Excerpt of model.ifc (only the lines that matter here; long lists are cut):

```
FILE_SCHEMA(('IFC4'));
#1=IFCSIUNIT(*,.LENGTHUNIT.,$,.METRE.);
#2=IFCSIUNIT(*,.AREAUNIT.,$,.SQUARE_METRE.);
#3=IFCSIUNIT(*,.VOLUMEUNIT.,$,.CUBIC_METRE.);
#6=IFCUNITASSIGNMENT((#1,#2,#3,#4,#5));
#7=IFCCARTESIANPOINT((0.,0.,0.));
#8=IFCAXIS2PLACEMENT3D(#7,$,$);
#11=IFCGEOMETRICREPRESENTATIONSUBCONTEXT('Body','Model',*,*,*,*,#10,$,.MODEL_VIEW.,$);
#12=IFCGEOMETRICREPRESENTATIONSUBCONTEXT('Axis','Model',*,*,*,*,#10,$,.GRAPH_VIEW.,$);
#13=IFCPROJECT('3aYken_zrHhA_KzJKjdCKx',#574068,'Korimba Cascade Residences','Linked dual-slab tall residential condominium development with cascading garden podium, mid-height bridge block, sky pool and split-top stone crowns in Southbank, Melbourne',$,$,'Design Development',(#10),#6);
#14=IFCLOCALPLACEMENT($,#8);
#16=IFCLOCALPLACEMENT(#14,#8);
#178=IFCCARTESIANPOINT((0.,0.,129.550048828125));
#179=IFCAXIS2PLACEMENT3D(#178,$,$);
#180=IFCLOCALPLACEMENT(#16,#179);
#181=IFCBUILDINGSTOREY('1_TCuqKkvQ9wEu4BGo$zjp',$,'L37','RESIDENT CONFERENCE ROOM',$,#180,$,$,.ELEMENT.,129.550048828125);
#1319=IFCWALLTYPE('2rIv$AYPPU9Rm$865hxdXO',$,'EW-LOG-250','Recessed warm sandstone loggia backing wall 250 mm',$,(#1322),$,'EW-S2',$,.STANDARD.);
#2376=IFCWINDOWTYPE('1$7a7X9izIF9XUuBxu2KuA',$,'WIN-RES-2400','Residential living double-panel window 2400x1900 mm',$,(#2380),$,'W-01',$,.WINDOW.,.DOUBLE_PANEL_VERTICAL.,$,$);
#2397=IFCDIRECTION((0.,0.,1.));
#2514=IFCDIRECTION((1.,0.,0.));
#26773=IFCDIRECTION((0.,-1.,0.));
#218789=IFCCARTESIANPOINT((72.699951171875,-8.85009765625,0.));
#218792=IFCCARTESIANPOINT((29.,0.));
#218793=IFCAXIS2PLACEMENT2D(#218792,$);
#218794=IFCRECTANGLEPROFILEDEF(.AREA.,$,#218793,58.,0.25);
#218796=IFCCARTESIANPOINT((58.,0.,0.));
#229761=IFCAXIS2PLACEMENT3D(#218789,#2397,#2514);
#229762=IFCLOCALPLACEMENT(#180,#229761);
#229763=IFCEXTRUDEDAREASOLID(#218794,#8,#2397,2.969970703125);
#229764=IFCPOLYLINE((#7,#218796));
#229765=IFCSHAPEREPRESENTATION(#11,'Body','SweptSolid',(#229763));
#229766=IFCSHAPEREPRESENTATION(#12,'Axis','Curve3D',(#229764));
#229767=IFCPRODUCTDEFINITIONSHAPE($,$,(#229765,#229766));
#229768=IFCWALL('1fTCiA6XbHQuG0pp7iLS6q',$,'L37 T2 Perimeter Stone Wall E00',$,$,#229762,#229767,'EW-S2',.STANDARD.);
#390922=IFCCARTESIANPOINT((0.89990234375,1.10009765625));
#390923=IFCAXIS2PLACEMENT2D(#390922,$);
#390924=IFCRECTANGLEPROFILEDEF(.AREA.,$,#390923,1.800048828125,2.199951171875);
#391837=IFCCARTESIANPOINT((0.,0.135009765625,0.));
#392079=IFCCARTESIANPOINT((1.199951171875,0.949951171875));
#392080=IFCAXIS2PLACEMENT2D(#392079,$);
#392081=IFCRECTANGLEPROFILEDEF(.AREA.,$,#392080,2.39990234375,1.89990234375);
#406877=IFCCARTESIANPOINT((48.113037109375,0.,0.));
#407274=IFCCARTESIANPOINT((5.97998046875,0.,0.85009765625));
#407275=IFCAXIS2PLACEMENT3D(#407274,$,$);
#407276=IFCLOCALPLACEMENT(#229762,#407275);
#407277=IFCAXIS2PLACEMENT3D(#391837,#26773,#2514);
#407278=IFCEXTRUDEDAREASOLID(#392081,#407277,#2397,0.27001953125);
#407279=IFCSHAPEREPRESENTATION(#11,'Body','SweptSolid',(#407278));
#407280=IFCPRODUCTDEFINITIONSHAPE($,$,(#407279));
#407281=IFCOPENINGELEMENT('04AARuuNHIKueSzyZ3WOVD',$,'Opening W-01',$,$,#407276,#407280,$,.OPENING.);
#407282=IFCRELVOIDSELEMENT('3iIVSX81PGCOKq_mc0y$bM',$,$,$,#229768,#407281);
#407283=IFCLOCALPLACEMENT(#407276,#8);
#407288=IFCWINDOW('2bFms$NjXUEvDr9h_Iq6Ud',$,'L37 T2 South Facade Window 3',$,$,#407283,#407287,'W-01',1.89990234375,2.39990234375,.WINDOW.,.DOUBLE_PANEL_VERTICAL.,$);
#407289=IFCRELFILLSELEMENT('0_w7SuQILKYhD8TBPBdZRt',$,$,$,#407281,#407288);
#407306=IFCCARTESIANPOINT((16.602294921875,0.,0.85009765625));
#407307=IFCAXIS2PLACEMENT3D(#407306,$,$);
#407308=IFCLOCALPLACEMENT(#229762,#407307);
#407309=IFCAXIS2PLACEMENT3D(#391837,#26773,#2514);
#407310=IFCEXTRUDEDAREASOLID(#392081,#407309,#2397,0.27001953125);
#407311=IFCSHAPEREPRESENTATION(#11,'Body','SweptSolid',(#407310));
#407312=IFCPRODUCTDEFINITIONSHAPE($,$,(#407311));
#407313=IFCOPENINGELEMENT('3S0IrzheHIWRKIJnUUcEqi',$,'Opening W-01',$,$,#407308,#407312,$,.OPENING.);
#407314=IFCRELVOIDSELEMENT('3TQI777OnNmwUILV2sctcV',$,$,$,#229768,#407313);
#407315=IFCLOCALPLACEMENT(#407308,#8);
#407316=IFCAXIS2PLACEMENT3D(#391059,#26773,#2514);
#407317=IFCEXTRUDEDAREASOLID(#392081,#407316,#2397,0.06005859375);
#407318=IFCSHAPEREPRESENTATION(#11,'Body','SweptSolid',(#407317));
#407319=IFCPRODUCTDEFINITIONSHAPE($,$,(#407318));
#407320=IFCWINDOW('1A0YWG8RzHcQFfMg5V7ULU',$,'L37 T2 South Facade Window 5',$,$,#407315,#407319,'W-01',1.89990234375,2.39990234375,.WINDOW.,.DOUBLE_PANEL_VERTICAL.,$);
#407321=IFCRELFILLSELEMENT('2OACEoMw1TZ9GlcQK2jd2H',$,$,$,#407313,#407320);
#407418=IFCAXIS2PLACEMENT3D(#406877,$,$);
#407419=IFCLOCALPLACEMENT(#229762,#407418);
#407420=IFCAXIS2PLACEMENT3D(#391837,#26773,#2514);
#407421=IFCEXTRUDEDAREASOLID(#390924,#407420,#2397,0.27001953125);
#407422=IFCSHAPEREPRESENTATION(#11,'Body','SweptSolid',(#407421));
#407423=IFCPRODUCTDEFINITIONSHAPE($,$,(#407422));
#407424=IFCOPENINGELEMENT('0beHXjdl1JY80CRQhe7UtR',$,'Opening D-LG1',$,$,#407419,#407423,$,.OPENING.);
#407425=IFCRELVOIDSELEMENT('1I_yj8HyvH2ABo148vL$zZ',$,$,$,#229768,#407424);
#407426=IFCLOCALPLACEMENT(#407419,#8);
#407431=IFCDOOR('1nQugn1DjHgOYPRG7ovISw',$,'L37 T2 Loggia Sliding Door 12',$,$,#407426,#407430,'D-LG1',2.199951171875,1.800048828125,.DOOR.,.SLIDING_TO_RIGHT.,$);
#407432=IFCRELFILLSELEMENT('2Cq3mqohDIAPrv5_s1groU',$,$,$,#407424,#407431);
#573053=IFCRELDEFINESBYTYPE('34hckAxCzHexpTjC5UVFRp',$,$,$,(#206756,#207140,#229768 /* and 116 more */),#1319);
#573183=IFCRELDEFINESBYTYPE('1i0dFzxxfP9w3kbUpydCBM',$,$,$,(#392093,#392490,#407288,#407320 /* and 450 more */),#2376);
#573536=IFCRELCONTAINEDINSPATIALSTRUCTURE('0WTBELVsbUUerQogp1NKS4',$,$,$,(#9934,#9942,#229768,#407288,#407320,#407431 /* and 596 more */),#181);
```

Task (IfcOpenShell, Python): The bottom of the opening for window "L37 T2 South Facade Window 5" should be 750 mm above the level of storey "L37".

```python
import numpy as np
import ifcopenshell
import ifcopenshell.api.geometry
import ifcopenshell.geom
import ifcopenshell.util.element
import ifcopenshell.util.placement
import ifcopenshell.util.shape
import ifcopenshell.util.unit

model = ifcopenshell.open("model.ifc")
unit_scale = ifcopenshell.util.unit.calculate_unit_scale(model)

window = model.by_guid("1A0YWG8RzHcQFfMg5V7ULU")
opening = window.FillsVoids[0].RelatingOpeningElement
storey = ifcopenshell.util.element.get_container(window, ifc_class="IfcBuildingStorey")
level = ifcopenshell.util.placement.get_local_placement(storey.ObjectPlacement)[2, 3]

# The opening's origin need not be at the sill, so measure its lowest point.
shape = ifcopenshell.geom.create_shape(ifcopenshell.geom.settings(), opening)
bottom = ifcopenshell.util.shape.get_shape_bottom_elevation(shape, shape.geometry) / unit_scale
dz = level + 0.75 / unit_scale - bottom

shift = np.array([0.0, 0.0, dz])
# The window is placed relative to its opening, so it follows when the opening moves.
matrix = ifcopenshell.util.placement.get_local_placement(opening.ObjectPlacement)
matrix[:3, 3] += shift
ifcopenshell.api.geometry.edit_object_placement(
    model, product=opening, matrix=matrix, is_si=False, should_transform_children=True
)

print(f"moved by {dz * unit_scale:+.3f} m")

model.write("model_updated.ifc")
```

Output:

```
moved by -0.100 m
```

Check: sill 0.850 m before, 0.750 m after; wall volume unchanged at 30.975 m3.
